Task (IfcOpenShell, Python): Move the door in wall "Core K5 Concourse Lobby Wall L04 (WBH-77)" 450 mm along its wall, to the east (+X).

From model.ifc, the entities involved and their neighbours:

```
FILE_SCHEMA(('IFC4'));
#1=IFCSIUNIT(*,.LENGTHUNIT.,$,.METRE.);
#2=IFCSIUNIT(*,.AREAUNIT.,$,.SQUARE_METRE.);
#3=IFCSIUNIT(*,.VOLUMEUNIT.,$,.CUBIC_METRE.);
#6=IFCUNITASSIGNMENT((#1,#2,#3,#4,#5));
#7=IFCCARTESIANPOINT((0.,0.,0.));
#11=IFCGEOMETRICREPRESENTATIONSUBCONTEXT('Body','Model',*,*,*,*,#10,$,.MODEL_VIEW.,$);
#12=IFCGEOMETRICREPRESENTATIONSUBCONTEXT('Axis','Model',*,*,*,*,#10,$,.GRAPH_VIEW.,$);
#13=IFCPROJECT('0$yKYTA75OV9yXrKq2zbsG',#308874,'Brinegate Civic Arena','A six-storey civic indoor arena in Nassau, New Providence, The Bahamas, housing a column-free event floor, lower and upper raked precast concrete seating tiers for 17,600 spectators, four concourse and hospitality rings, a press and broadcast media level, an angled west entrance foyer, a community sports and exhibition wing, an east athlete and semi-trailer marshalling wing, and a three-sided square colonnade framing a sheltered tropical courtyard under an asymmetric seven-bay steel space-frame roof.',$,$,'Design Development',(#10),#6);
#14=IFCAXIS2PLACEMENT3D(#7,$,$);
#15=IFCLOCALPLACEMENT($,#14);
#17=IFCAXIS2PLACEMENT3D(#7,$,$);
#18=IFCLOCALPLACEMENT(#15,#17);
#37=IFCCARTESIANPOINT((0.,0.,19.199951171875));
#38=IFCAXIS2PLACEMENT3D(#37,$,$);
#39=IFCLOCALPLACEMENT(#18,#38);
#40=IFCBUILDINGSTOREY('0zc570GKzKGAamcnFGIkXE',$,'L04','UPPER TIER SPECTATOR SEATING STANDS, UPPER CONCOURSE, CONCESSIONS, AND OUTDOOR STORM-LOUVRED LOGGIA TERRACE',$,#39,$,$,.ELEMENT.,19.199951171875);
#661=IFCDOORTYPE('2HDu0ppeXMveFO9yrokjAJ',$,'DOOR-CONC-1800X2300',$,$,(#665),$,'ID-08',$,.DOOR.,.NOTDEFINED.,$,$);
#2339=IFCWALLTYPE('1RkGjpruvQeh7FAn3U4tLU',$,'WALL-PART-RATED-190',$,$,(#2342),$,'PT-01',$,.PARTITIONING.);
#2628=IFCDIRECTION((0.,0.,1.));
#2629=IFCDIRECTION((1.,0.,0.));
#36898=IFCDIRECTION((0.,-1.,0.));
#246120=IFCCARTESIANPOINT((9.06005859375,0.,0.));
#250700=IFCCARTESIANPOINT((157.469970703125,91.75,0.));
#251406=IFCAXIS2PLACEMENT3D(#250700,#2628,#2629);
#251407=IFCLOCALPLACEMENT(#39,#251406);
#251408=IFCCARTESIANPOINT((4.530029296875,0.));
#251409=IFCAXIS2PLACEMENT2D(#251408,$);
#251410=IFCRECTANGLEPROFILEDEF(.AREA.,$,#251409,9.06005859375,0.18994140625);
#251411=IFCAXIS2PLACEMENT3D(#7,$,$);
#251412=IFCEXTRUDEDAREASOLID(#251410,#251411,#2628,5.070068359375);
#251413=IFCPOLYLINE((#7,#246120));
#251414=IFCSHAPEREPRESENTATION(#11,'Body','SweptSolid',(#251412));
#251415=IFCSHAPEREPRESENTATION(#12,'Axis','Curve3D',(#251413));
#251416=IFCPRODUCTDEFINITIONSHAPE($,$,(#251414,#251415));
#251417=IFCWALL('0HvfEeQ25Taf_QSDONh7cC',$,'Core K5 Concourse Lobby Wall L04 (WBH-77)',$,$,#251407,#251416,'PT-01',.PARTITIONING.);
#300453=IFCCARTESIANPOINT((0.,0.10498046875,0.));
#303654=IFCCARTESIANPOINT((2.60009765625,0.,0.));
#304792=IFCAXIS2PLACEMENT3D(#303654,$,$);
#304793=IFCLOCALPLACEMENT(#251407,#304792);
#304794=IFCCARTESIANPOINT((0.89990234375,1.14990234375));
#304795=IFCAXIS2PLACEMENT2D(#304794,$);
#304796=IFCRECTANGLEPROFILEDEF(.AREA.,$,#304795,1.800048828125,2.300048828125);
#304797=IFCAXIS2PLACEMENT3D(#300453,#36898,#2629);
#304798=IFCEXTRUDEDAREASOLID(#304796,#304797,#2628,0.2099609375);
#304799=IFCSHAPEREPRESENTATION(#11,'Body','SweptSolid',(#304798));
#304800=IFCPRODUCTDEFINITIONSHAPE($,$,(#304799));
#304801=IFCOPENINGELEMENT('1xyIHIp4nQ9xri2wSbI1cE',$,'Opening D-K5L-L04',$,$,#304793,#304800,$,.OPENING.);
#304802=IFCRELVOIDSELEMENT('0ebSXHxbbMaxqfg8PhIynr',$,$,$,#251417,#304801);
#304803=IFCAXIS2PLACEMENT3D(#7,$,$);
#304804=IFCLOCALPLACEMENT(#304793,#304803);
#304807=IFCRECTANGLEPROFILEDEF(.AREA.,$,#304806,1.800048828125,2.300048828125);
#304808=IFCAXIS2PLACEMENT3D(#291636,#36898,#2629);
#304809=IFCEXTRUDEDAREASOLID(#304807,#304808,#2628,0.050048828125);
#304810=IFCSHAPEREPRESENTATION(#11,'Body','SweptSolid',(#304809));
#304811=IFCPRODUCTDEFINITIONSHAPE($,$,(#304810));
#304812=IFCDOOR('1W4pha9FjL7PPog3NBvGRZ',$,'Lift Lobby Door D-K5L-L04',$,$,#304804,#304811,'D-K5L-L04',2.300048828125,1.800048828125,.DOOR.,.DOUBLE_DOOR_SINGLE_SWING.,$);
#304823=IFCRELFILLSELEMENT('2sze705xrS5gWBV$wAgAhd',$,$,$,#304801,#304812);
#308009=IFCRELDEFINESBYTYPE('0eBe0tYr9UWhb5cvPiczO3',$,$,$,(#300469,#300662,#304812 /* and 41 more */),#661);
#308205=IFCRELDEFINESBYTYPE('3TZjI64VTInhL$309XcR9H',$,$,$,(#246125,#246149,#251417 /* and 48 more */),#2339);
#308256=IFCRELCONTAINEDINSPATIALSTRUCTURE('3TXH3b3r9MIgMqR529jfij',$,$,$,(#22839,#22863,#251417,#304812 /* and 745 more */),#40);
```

```python
import ifcopenshell
import ifcopenshell.api.geometry
import ifcopenshell.util.placement

model = ifcopenshell.open("model.ifc")

door = model.by_id(304812)
opening = door.FillsVoids[0].RelatingOpeningElement
wall = opening.VoidsElements[0].RelatingBuildingElement

wall_matrix = ifcopenshell.util.placement.get_local_placement(wall.ObjectPlacement)
shift = wall_matrix[:3, 0] * 0.45
before = ifcopenshell.util.placement.get_local_placement(door.ObjectPlacement)[:3, 3].copy()

# The door is placed relative to its opening, so it follows when the opening moves.
matrix = ifcopenshell.util.placement.get_local_placement(opening.ObjectPlacement)
matrix[:3, 3] += shift
ifcopenshell.api.geometry.edit_object_placement(
    model, product=opening, matrix=matrix, is_si=False, should_transform_children=True
)

after = ifcopenshell.util.placement.get_local_placement(door.ObjectPlacement)[:3, 3]
print("door moved by", (after - before).round(3) + 0.0)

model.write("model-out.ifc")
```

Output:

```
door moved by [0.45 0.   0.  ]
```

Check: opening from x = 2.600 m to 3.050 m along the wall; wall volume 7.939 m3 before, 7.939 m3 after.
